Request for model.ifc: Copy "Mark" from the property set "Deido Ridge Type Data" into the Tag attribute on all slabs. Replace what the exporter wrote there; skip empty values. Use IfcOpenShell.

First a look at what the model holds.

```python
import ifcopenshell
import ifcopenshell.util.element

model = ifcopenshell.open("model.ifc")
print(model.schema)
slabs = model.by_type("IfcSlab")
print(len(slabs), "slabs")
for e in slabs[:8]:
    source = ifcopenshell.util.element.get_pset(e, "Deido Ridge Type Data", "Mark")
    target = e.Tag
    print(e.id(), repr(source), repr(target), sep=" | ")
```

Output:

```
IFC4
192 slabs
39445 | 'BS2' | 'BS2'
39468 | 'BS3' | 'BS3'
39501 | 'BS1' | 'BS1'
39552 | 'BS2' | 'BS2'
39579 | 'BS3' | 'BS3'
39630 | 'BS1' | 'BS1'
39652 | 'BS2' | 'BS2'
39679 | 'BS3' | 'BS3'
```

```python
import ifcopenshell
import ifcopenshell.util.element

model = ifcopenshell.open("model.ifc")

count = 0
for e in model.by_type("IfcSlab"):
    value = ifcopenshell.util.element.get_pset(e, "Deido Ridge Type Data", "Mark")
    current = e.Tag
    if not value or not value.strip() or current == value:
        continue
    e.Tag = value
    count += 1

print(count, "slabs updated")

model.write("model-out.ifc")
```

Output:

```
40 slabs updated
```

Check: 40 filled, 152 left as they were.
